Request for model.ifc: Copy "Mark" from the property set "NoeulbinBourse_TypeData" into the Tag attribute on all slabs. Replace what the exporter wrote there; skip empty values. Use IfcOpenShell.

First a look at what the model holds.

```python
import ifcopenshell
import ifcopenshell.util.element

model = ifcopenshell.open("model.ifc")
print(model.schema)
slabs = model.by_type("IfcSlab")
print(len(slabs), "slabs")
for e in slabs[:8]:
    source = ifcopenshell.util.element.get_pset(e, "NoeulbinBourse_TypeData", "Mark")
    target = e.Tag
    print(e.id(), repr(source), repr(target), sep=" | ")
```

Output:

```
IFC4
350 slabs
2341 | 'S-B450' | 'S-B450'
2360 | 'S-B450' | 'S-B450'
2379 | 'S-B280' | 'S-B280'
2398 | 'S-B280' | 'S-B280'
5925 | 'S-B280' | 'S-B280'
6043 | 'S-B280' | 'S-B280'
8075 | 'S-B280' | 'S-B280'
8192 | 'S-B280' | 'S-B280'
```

```python
import ifcopenshell
import ifcopenshell.util.element

model = ifcopenshell.open("model.ifc")

count = 0
for e in model.by_type("IfcSlab"):
    value = ifcopenshell.util.element.get_pset(e, "NoeulbinBourse_TypeData", "Mark")
    current = e.Tag
    if not value or not value.strip() or current == value:
        continue
    e.Tag = value
    count += 1

print(count, "slabs updated")

model.write("model-out.ifc")
```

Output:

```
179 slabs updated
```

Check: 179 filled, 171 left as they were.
